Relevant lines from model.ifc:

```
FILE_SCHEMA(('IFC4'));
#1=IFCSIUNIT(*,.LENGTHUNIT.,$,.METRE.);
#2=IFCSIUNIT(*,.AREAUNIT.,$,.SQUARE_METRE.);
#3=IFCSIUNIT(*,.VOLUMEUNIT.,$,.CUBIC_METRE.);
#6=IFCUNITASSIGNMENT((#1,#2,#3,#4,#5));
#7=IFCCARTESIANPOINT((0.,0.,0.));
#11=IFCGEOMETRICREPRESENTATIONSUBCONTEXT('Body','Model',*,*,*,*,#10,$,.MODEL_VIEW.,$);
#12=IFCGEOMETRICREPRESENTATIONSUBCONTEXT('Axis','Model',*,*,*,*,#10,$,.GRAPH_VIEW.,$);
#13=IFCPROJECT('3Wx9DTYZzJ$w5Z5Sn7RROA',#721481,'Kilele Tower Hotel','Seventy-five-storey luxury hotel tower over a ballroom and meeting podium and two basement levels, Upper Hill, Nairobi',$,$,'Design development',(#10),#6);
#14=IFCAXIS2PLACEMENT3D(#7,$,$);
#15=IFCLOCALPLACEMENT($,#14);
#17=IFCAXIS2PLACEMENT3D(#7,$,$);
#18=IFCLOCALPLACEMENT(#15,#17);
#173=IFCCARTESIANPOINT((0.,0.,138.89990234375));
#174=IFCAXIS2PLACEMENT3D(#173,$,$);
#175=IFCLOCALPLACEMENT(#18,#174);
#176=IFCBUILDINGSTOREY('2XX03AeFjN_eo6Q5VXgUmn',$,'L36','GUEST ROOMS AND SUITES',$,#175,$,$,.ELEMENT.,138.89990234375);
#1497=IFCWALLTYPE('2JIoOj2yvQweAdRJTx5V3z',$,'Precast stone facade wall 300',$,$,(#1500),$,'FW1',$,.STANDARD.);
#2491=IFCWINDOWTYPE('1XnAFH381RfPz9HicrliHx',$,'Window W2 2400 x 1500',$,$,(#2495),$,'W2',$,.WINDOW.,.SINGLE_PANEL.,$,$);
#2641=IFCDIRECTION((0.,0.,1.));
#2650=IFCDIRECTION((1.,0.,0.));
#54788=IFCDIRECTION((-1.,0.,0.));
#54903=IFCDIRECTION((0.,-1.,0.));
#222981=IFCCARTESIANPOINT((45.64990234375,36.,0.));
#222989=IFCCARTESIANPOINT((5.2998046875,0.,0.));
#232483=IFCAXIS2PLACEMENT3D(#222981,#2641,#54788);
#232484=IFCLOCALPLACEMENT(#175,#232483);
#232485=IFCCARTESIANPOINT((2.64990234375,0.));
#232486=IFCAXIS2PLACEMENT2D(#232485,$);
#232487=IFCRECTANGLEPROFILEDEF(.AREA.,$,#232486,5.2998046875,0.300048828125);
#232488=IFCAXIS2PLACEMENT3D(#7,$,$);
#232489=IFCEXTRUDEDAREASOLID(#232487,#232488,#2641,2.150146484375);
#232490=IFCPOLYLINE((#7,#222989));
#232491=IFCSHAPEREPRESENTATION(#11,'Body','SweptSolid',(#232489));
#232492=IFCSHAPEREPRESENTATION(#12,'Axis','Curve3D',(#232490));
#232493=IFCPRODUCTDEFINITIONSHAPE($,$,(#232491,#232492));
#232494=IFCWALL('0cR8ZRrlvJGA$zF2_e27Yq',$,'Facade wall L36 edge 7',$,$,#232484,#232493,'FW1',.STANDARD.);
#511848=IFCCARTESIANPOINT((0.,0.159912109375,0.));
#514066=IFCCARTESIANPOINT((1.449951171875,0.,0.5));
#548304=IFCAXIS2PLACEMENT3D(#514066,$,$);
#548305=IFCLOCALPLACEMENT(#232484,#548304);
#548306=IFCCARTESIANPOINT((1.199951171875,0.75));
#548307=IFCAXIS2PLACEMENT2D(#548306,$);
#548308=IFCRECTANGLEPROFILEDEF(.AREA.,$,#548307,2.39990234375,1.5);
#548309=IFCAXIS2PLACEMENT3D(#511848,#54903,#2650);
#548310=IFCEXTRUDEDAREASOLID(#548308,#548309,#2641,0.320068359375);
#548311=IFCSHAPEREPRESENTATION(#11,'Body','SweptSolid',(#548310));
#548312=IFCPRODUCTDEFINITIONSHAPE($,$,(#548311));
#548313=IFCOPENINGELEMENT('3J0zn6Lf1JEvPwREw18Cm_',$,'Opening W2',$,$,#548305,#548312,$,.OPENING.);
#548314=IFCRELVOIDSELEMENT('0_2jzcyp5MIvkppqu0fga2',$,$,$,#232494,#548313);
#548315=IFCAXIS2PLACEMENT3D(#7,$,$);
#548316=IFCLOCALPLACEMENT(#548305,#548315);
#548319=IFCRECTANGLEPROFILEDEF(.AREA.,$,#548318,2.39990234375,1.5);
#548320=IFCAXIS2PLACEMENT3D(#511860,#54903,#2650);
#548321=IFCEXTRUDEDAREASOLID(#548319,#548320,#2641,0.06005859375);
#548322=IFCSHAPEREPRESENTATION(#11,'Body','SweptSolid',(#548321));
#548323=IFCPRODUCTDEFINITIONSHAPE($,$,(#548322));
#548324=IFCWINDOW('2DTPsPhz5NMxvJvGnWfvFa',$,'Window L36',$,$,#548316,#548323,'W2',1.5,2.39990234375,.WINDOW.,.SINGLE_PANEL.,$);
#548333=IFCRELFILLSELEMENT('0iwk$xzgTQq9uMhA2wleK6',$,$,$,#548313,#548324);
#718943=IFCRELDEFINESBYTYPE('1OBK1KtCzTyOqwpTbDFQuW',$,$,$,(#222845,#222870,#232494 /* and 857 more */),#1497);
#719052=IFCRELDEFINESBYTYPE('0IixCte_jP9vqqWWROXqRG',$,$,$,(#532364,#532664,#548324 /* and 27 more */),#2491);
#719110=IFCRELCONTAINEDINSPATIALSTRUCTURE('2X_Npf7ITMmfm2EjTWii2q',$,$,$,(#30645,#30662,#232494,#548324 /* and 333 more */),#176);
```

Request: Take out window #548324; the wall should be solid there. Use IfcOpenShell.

```python
import ifcopenshell
import ifcopenshell.api.feature
import ifcopenshell.api.root
import ifcopenshell.geom
import ifcopenshell.util.shape

model = ifcopenshell.open("model.ifc")
settings = ifcopenshell.geom.settings()


def volume(element):
    """Net volume in cubic metres, openings subtracted."""
    shape = ifcopenshell.geom.create_shape(settings, element)
    return ifcopenshell.util.shape.get_volume(shape.geometry)


window = model.by_guid("2DTPsPhz5NMxvJvGnWfvFa")
opening = window.FillsVoids[0].RelatingOpeningElement
wall = opening.VoidsElements[0].RelatingBuildingElement
before = volume(wall)

ifcopenshell.api.root.remove_product(model, product=window)
ifcopenshell.api.feature.remove_feature(model, feature=opening)

after = volume(wall)

print(f"wall volume {before:.3f} -> {after:.3f} m3")

model.write("model_rev.ifc")
```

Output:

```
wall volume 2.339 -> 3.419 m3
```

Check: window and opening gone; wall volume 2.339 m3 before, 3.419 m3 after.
